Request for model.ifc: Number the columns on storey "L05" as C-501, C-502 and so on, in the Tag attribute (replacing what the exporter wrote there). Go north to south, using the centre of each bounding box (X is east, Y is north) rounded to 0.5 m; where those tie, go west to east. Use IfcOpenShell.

First a look at what the model holds.

```python
import ifcopenshell
import ifcopenshell.util.element
import ifcopenshell.util.placement

model = ifcopenshell.open("model.ifc")
print(model.schema)
storey = next(s for s in model.by_type("IfcBuildingStorey") if s.Name == "L05")
columns = [e for e in ifcopenshell.util.element.get_decomposition(storey) if e.is_a("IfcColumn")]
for e in sorted(columns, key=lambda e: e.id()):
    origin = ifcopenshell.util.placement.get_local_placement(e.ObjectPlacement)[:3, 3]
    print(e.id(), e.Tag, e.Name, origin.round(2) + 0.0, sep=" | ")
```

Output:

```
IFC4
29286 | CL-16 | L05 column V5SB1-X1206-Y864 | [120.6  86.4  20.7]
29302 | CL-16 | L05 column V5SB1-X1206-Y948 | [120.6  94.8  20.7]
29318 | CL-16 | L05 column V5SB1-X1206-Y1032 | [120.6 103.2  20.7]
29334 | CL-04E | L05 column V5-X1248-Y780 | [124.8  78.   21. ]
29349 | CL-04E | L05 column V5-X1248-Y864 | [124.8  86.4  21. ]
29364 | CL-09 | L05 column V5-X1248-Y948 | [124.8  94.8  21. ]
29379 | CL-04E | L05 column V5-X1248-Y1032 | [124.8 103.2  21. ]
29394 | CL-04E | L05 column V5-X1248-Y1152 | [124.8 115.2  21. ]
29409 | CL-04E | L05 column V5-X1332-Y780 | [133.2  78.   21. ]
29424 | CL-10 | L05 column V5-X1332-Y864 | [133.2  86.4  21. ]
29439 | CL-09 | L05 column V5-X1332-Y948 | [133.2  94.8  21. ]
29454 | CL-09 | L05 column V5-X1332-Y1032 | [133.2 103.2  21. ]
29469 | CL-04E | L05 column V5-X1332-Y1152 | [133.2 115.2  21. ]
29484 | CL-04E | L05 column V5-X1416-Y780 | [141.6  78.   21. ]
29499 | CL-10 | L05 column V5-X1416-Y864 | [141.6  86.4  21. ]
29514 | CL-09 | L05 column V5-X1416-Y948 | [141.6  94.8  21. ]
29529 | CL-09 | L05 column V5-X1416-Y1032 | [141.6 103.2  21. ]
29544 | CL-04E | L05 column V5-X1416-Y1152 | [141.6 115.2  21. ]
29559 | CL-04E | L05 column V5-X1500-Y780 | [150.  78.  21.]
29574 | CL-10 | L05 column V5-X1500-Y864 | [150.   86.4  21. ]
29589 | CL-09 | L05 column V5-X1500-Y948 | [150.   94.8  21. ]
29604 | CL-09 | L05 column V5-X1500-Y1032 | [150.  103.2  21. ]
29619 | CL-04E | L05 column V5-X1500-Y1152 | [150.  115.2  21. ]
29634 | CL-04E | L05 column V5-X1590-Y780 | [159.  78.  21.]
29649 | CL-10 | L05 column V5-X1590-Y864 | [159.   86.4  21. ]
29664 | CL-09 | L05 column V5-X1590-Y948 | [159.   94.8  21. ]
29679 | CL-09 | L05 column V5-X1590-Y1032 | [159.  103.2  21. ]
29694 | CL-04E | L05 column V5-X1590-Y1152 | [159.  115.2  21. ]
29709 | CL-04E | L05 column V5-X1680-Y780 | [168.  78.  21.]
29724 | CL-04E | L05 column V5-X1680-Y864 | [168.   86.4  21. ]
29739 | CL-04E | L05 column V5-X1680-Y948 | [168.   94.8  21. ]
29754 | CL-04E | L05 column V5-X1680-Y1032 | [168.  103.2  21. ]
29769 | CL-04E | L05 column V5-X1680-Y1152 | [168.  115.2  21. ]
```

```python
import ifcopenshell
import ifcopenshell.geom
import ifcopenshell.util.element
import ifcopenshell.util.shape

model = ifcopenshell.open("model.ifc")
settings = ifcopenshell.geom.settings()
settings.set("use-world-coords", True)


def centre(element):
    shape = ifcopenshell.geom.create_shape(settings, element)
    return ifcopenshell.util.shape.get_bbox_centroid(shape.geometry)


storey = next(s for s in model.by_type("IfcBuildingStorey") if s.Name == "L05")
columns = [e for e in ifcopenshell.util.element.get_decomposition(storey) if e.is_a("IfcColumn")]

# Insertion points can sit at a corner or the storey origin, so sort by the geometry (in metres).
centres = {e: centre(e) for e in columns}
columns.sort(key=lambda e: (-round(centres[e][1] / 0.5), centres[e][0]))

for i, e in enumerate(columns, start=1):
    number = f"C-5{i:02d}"
    e.Tag = number
    print(e.id(), number)

model.write("model_updated.ifc")
```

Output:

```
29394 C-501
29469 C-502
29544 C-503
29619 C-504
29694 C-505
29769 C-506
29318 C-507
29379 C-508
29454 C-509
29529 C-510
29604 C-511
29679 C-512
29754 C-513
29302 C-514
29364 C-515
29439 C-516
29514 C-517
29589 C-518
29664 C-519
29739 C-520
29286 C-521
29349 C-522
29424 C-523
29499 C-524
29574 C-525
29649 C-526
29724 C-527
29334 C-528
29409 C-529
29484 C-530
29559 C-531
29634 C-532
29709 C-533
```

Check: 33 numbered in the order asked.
